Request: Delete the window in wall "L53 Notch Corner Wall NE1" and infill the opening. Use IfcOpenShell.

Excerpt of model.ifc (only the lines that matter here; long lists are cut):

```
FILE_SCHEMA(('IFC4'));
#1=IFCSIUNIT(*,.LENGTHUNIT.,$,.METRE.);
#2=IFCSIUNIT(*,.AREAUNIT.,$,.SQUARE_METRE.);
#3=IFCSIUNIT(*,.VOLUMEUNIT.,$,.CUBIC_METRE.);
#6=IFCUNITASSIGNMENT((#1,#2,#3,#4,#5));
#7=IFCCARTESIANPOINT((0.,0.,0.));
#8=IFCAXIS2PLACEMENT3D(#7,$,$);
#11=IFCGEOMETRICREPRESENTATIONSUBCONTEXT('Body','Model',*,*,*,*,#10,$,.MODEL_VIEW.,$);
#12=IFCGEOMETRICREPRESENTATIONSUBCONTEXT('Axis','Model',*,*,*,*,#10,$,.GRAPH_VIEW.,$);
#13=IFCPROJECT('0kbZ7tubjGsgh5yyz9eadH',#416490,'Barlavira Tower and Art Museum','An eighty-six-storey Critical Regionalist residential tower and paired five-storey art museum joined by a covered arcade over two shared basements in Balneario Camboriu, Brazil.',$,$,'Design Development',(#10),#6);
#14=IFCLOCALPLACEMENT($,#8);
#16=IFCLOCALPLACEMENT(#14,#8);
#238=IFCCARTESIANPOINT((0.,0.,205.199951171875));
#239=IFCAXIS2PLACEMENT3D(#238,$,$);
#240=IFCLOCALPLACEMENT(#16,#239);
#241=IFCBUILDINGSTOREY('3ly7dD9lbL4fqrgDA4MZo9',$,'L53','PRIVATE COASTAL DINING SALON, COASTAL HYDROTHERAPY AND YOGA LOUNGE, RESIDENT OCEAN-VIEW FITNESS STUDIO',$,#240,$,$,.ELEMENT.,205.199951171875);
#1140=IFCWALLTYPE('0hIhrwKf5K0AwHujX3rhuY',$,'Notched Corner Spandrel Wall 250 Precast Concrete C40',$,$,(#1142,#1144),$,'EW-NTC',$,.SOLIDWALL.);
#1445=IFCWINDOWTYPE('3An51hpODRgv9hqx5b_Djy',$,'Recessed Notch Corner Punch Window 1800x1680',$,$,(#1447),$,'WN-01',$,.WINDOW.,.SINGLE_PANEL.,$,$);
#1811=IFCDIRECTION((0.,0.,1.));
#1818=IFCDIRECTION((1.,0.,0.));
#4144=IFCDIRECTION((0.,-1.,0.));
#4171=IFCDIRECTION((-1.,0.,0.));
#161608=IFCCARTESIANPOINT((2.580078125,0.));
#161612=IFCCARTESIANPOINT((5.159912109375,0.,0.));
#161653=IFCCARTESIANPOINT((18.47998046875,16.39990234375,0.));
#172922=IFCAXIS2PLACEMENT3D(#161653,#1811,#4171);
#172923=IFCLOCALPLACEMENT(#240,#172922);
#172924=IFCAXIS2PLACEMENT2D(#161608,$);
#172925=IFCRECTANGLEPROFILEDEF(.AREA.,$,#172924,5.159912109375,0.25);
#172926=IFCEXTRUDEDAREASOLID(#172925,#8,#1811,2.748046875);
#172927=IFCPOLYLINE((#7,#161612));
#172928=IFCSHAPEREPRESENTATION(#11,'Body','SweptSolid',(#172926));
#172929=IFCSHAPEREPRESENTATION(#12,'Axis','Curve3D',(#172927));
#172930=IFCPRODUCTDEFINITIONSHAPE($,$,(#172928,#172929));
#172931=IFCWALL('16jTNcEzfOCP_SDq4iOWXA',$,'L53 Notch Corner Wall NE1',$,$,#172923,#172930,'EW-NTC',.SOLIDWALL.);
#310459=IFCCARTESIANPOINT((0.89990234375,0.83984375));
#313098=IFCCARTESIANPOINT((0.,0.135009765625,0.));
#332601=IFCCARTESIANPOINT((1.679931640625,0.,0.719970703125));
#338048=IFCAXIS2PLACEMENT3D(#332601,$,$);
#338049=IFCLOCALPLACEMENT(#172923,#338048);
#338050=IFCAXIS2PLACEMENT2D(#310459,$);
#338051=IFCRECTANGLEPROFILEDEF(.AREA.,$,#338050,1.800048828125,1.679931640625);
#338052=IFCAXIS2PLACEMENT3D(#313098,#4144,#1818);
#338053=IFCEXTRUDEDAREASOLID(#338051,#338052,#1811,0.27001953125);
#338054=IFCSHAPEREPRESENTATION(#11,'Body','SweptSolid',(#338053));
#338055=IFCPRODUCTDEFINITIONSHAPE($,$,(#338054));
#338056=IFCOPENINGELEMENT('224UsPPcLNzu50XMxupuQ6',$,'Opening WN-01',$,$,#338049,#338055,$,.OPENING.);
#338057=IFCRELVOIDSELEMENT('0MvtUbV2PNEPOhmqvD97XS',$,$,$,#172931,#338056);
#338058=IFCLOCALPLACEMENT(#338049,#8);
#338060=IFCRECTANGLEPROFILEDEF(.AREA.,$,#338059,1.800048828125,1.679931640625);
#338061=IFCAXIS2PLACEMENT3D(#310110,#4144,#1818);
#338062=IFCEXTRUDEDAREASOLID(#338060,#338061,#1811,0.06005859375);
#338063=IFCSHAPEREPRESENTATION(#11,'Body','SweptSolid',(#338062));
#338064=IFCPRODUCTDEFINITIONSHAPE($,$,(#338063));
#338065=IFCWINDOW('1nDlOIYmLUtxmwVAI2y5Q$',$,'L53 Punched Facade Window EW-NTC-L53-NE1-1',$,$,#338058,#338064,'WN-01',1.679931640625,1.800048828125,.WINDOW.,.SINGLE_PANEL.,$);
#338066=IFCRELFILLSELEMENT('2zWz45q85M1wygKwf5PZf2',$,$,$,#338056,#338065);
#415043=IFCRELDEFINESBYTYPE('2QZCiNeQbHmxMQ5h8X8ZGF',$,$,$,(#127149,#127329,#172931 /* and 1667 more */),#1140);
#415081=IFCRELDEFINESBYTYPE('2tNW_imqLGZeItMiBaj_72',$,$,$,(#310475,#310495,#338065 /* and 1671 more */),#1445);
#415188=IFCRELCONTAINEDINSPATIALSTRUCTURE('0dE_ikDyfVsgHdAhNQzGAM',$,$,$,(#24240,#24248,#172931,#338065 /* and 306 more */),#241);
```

```python
import ifcopenshell
import ifcopenshell.api.feature
import ifcopenshell.api.root
import ifcopenshell.geom
import ifcopenshell.util.shape

model = ifcopenshell.open("model.ifc")
settings = ifcopenshell.geom.settings()


def volume(element):
    """Net volume in cubic metres, openings subtracted."""
    shape = ifcopenshell.geom.create_shape(settings, element)
    return ifcopenshell.util.shape.get_volume(shape.geometry)


window = model.by_id(338065)
opening = window.FillsVoids[0].RelatingOpeningElement
wall = opening.VoidsElements[0].RelatingBuildingElement
before = volume(wall)

ifcopenshell.api.root.remove_product(model, product=window)
ifcopenshell.api.feature.remove_feature(model, feature=opening)

after = volume(wall)

print(f"wall volume {before:.3f} -> {after:.3f} m3")

model.write("model_updated.ifc")
```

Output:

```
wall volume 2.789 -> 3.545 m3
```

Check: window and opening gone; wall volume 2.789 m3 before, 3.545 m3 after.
